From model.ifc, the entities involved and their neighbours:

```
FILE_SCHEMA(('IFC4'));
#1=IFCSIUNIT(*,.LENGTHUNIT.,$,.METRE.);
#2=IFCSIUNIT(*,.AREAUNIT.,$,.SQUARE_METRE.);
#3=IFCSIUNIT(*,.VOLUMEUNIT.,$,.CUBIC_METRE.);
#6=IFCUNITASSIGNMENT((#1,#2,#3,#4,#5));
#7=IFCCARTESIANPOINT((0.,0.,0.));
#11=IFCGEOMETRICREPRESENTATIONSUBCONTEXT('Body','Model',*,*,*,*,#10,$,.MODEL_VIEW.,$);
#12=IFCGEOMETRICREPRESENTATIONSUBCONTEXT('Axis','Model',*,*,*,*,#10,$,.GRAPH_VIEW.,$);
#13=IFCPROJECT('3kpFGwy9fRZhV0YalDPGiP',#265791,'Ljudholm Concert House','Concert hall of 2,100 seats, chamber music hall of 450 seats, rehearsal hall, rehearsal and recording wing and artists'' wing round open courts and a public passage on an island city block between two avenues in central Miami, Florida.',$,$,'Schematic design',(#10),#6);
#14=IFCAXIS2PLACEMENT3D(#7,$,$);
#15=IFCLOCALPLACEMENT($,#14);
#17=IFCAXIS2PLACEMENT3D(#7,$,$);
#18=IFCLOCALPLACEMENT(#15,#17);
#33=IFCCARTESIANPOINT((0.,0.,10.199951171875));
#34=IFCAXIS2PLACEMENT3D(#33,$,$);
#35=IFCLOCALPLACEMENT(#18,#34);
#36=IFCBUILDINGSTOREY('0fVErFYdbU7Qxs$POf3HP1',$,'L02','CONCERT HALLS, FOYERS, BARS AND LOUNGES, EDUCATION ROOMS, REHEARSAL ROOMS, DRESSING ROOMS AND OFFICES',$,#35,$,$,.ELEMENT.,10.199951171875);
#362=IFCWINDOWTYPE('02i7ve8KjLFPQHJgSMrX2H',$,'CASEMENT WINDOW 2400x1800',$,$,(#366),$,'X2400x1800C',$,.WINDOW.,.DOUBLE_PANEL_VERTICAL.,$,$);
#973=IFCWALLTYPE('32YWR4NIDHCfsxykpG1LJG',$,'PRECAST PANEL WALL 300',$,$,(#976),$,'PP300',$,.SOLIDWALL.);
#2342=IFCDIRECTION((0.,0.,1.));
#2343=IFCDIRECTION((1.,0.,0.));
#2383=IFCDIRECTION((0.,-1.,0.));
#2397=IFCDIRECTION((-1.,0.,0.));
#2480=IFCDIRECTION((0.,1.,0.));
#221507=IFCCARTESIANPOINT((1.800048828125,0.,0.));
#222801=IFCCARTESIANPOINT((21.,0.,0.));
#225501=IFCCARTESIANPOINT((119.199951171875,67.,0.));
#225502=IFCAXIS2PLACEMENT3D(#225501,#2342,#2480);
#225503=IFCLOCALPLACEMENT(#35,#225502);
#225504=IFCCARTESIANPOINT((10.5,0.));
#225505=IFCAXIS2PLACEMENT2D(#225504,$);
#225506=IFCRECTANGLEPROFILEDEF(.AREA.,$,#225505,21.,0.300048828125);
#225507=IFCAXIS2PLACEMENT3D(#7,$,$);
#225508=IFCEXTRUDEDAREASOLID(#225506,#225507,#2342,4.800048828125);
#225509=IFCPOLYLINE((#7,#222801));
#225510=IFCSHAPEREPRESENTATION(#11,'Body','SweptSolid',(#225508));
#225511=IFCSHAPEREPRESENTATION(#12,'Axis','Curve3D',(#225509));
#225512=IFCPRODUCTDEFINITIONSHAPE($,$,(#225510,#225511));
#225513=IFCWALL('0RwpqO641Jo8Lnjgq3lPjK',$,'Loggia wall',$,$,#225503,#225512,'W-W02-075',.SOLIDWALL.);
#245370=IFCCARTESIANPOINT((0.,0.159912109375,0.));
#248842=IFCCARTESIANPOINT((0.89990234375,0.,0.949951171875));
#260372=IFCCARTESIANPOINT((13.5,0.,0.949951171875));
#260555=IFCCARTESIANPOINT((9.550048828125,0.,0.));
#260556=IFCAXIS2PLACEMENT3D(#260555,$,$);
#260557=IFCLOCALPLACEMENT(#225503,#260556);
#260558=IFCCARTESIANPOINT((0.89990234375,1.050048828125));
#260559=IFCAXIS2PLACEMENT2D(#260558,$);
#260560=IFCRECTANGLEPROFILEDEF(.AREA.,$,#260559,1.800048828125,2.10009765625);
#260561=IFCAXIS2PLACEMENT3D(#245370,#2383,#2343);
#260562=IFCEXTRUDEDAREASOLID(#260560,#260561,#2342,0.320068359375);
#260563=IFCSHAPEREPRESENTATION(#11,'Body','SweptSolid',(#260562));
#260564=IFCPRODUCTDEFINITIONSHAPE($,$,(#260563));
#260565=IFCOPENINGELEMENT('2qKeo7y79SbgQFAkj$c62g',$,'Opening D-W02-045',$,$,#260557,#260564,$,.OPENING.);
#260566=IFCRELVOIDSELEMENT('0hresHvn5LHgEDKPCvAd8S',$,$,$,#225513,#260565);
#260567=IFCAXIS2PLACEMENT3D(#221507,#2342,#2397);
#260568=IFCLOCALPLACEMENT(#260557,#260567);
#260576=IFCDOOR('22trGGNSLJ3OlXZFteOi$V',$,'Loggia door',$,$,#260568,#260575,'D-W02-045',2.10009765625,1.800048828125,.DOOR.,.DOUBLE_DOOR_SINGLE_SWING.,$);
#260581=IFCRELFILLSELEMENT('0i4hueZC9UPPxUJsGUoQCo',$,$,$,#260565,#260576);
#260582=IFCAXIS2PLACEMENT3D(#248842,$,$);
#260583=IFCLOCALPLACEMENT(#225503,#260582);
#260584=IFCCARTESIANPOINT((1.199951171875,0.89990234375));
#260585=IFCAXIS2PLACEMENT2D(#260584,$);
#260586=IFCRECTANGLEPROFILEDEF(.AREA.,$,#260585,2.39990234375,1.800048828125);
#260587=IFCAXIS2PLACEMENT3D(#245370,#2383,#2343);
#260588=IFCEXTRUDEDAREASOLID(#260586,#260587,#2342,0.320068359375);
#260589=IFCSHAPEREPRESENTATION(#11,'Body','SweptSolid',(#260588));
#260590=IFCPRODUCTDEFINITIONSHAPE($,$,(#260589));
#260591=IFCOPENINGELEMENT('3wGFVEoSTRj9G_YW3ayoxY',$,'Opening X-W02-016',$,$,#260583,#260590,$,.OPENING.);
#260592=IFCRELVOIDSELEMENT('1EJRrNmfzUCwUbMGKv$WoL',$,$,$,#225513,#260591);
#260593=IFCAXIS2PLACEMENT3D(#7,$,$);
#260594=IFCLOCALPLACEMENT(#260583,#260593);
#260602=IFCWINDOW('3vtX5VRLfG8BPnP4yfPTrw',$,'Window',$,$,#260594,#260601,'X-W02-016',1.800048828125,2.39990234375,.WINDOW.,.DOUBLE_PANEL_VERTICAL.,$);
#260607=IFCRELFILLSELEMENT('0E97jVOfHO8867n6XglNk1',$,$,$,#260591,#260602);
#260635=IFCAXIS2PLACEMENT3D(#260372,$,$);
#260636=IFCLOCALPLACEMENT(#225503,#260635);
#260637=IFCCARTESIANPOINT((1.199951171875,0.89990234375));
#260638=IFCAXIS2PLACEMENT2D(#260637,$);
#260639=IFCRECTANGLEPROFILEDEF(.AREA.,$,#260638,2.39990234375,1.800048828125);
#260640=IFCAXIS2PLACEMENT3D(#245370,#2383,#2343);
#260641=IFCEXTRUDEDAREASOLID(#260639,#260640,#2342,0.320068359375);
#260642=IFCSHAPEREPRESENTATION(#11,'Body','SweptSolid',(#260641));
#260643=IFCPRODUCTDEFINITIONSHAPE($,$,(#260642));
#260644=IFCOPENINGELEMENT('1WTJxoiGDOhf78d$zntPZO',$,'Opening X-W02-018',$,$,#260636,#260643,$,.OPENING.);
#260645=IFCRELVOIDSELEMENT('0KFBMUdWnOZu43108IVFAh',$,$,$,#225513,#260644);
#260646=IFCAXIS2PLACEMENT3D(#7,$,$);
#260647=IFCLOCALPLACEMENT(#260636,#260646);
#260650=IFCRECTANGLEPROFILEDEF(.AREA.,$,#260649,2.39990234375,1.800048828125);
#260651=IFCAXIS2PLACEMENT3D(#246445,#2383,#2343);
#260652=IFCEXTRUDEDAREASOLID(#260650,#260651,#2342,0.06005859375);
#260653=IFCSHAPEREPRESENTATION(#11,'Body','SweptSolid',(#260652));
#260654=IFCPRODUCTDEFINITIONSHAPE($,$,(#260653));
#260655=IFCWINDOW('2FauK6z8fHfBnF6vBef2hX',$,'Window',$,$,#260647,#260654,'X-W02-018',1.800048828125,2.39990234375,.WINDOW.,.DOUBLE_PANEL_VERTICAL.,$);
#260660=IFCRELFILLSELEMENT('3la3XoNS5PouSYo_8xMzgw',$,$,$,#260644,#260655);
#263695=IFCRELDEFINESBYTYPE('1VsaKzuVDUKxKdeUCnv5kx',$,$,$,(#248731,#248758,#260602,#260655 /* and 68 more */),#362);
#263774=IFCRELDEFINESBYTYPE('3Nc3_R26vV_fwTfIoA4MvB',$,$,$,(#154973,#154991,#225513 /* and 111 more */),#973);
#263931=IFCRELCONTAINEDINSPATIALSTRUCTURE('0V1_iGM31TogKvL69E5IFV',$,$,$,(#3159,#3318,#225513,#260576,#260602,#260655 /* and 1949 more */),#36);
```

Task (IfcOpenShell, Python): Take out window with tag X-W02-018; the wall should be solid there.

```python
import ifcopenshell
import ifcopenshell.api.feature
import ifcopenshell.api.root
import ifcopenshell.geom
import ifcopenshell.util.shape

model = ifcopenshell.open("model.ifc")
settings = ifcopenshell.geom.settings()


def volume(element):
    """Net volume in cubic metres, openings subtracted."""
    shape = ifcopenshell.geom.create_shape(settings, element)
    return ifcopenshell.util.shape.get_volume(shape.geometry)


window = model.by_guid("2FauK6z8fHfBnF6vBef2hX")
opening = window.FillsVoids[0].RelatingOpeningElement
wall = opening.VoidsElements[0].RelatingBuildingElement
before = volume(wall)

ifcopenshell.api.root.remove_product(model, product=window)
ifcopenshell.api.feature.remove_feature(model, feature=opening)

after = volume(wall)

print(f"wall volume {before:.3f} -> {after:.3f} m3")

model.write("model_v2.ifc")
```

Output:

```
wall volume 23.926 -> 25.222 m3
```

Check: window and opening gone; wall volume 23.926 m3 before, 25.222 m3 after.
